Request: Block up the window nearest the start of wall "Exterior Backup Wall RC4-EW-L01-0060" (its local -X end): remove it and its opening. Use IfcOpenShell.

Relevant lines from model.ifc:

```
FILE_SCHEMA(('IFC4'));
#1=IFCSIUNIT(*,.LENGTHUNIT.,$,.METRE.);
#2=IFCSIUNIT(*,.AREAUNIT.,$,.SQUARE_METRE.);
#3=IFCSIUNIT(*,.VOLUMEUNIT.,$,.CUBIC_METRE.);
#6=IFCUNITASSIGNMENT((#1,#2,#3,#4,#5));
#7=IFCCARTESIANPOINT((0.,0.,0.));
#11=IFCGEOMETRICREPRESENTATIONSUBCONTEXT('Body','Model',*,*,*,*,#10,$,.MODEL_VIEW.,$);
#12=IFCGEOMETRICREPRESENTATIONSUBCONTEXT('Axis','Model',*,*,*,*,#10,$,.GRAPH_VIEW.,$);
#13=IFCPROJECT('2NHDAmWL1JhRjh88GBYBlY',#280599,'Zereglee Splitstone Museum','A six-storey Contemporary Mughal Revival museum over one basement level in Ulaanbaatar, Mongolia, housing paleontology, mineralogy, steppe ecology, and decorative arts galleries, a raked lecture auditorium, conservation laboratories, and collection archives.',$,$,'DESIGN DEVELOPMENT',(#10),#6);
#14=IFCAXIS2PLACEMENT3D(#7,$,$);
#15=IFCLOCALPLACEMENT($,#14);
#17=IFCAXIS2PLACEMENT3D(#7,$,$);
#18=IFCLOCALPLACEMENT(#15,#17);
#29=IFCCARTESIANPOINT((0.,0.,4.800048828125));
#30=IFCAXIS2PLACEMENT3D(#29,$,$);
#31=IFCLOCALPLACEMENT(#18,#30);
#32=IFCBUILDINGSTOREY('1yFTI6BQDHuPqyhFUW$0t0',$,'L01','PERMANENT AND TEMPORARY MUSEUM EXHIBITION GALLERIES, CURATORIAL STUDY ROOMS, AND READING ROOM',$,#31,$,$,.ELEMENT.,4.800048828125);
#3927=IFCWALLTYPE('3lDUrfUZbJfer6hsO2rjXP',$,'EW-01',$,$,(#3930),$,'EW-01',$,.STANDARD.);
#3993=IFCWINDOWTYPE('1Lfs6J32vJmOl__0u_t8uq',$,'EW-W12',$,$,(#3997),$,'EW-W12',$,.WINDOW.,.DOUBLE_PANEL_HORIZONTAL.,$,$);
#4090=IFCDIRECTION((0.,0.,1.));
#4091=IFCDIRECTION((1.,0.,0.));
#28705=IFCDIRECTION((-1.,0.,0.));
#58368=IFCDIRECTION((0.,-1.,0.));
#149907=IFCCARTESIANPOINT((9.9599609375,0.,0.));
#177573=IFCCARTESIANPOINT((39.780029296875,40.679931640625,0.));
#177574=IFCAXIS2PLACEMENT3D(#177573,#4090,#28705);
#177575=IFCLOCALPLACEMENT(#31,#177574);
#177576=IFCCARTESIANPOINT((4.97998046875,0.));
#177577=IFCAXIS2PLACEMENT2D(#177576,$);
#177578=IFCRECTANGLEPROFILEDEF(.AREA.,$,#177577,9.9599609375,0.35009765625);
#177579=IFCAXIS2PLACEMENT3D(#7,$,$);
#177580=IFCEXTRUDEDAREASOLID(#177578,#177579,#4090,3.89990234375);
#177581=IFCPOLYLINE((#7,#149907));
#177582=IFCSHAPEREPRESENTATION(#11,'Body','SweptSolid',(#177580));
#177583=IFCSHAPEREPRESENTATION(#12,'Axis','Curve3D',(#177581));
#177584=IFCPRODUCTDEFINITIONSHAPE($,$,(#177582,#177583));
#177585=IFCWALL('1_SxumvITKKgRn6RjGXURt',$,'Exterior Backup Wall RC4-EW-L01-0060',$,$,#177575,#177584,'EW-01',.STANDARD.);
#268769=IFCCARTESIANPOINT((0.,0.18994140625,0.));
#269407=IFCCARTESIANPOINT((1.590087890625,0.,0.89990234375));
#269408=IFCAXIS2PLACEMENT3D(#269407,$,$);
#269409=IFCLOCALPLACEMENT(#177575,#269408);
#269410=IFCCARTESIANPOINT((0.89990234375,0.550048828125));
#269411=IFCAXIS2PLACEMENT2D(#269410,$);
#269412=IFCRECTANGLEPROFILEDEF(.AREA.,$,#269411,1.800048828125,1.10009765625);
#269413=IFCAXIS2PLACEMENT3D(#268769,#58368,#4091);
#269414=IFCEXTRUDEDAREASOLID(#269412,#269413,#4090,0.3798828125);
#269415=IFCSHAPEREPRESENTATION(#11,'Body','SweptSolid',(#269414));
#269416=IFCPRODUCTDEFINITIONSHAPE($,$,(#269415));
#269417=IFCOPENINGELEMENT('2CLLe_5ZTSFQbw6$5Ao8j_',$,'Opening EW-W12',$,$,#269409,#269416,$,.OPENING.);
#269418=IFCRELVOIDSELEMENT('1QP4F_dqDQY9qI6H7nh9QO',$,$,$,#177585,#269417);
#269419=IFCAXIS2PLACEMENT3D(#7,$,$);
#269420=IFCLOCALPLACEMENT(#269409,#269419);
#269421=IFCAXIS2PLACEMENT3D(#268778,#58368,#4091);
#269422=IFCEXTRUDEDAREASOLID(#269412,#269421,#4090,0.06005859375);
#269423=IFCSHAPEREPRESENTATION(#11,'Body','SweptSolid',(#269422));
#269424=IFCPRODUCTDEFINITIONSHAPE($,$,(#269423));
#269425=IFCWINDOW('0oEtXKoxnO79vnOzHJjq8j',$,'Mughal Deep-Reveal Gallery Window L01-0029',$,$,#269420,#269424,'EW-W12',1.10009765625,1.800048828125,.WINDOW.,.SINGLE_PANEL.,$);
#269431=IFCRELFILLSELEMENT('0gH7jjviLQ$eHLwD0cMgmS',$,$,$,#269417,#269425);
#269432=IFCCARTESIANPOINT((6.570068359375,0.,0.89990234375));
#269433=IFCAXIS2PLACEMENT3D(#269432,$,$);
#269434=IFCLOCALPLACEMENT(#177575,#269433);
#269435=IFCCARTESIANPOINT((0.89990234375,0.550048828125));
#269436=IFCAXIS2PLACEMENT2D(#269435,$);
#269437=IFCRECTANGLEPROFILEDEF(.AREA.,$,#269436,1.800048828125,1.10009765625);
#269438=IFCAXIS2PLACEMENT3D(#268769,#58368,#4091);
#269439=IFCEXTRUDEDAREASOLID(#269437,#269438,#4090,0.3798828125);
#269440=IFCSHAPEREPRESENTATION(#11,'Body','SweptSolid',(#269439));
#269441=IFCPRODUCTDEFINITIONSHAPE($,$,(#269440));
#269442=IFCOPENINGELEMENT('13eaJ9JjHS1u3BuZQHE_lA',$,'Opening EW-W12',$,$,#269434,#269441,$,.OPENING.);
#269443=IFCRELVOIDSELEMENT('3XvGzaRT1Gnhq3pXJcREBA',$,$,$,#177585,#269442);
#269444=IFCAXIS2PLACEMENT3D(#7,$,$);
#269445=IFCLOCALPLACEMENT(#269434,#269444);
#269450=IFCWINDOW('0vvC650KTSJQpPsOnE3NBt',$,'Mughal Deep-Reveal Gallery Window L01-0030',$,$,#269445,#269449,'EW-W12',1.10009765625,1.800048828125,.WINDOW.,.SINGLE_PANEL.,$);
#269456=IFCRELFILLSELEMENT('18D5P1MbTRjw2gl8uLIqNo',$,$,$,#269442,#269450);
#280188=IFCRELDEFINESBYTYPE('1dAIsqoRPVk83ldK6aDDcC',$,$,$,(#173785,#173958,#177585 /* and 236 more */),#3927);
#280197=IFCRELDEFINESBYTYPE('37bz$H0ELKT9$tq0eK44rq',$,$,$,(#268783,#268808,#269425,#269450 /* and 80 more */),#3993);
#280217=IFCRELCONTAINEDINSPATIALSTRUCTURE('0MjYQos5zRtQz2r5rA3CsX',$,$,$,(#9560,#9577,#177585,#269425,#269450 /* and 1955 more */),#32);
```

```python
import ifcopenshell
import ifcopenshell.api.feature
import ifcopenshell.api.root
import ifcopenshell.geom
import ifcopenshell.util.shape

model = ifcopenshell.open("model.ifc")
settings = ifcopenshell.geom.settings()


def volume(element):
    """Net volume in cubic metres, openings subtracted."""
    shape = ifcopenshell.geom.create_shape(settings, element)
    return ifcopenshell.util.shape.get_volume(shape.geometry)


window = model.by_guid("0oEtXKoxnO79vnOzHJjq8j")
opening = window.FillsVoids[0].RelatingOpeningElement
wall = opening.VoidsElements[0].RelatingBuildingElement
before = volume(wall)

ifcopenshell.api.root.remove_product(model, product=window)
ifcopenshell.api.feature.remove_feature(model, feature=opening)

after = volume(wall)

print(f"wall volume {before:.3f} -> {after:.3f} m3")

model.write("model-out.ifc")
```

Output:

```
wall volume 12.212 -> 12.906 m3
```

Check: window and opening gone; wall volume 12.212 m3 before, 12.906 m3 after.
